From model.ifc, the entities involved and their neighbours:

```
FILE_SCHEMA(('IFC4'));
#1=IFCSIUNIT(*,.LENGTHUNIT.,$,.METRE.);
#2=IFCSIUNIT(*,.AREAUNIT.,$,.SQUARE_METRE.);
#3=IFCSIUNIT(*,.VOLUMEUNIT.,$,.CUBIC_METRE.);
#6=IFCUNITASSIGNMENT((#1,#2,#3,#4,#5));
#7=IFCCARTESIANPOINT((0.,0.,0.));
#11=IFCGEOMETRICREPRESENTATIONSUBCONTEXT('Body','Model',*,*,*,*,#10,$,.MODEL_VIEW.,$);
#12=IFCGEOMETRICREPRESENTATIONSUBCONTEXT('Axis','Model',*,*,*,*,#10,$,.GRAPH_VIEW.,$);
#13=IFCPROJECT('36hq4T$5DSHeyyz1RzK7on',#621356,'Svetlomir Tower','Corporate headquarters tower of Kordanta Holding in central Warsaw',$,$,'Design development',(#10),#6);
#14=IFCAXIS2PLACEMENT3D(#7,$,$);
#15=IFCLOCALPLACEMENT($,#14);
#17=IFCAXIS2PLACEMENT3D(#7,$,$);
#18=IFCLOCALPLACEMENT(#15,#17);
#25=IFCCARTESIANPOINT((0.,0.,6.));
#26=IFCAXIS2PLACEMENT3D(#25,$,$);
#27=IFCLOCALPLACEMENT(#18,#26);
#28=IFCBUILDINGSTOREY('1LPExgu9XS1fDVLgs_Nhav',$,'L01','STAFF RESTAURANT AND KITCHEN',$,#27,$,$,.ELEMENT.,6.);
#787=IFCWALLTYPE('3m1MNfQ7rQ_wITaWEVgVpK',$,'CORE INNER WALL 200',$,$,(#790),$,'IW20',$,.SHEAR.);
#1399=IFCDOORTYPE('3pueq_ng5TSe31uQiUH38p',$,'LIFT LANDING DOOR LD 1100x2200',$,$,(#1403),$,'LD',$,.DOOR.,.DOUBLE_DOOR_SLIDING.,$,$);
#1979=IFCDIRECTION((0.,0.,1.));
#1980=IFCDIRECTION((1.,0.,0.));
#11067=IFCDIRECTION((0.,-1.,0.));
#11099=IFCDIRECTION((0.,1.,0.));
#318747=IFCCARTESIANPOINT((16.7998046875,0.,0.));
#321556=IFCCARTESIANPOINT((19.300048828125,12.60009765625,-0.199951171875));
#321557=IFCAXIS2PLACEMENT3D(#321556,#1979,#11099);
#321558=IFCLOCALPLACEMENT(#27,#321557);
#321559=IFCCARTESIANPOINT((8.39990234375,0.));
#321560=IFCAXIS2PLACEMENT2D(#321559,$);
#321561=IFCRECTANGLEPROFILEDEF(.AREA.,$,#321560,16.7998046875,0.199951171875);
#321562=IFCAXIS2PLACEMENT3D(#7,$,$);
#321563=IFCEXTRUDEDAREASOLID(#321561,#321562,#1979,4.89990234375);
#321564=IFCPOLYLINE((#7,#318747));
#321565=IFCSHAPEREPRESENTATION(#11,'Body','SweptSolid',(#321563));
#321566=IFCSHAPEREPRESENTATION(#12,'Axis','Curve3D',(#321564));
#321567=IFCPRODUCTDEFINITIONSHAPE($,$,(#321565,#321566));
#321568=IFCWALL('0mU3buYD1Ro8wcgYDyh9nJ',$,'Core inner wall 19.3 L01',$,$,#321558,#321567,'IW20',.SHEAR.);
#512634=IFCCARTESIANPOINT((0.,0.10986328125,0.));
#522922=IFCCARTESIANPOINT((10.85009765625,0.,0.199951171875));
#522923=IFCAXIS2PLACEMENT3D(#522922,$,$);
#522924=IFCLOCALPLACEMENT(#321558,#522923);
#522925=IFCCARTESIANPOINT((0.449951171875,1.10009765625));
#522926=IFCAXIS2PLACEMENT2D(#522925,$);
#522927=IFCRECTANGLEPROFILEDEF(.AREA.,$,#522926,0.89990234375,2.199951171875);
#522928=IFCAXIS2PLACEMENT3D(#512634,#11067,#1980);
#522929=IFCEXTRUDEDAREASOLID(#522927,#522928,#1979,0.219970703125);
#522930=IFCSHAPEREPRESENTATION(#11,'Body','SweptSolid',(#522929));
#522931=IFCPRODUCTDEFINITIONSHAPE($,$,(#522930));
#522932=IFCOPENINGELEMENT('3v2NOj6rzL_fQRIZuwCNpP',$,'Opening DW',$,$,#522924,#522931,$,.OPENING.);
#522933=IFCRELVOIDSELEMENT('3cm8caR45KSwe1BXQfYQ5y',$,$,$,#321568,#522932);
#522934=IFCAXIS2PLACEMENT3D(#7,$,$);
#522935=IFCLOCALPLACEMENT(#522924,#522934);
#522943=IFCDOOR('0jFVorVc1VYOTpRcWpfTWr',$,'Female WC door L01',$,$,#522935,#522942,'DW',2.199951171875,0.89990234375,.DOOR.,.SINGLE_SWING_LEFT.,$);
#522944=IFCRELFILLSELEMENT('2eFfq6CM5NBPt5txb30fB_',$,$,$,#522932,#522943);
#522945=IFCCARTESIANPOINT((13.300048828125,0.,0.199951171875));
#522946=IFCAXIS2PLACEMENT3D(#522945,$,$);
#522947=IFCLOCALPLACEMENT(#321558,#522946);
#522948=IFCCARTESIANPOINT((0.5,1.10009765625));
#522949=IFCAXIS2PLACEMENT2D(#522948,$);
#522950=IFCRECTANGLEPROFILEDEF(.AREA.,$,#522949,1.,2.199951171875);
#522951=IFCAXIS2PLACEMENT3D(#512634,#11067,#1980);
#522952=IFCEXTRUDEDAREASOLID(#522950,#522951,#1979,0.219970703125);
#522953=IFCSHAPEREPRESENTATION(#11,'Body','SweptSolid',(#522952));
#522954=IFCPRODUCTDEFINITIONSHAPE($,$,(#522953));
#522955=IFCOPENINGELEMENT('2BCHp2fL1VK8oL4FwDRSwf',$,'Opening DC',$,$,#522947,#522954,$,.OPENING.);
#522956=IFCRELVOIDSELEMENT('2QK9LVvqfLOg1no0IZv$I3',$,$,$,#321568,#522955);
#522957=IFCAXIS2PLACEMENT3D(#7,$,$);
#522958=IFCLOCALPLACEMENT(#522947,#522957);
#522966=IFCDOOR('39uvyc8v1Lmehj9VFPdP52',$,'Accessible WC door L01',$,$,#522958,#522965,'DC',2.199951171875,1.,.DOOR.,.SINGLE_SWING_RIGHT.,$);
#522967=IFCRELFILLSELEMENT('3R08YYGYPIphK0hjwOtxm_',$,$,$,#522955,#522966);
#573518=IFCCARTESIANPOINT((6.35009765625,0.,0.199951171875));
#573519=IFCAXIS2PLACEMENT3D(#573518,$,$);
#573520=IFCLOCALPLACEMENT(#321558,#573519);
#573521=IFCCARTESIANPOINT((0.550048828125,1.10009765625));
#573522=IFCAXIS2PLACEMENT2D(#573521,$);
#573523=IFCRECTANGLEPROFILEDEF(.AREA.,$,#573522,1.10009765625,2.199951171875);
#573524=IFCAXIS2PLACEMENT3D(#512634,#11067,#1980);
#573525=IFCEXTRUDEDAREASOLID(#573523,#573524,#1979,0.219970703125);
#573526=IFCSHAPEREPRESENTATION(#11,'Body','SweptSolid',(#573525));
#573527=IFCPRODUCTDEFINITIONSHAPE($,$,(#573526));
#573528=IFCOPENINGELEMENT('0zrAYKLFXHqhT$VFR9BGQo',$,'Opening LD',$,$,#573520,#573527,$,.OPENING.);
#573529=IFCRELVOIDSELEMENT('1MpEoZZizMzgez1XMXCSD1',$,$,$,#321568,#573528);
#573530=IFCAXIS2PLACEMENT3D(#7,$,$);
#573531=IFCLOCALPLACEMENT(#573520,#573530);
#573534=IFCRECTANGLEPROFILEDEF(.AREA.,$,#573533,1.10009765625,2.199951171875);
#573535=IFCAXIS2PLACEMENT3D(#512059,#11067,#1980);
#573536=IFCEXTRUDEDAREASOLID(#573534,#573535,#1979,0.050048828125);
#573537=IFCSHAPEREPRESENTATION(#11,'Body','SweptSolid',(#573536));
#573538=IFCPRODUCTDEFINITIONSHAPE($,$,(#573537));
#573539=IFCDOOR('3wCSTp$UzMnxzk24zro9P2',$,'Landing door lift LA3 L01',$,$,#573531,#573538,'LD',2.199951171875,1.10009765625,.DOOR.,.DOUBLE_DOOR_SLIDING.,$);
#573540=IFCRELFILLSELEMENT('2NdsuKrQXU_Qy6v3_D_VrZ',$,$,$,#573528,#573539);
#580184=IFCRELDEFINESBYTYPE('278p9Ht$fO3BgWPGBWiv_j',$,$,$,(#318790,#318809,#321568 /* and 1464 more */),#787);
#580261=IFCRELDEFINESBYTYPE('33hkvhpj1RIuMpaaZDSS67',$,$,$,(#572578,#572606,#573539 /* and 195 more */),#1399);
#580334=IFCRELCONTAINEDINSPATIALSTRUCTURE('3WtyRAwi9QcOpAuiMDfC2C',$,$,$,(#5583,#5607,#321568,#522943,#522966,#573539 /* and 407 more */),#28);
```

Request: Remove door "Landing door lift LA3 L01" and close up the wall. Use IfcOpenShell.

```python
import ifcopenshell
import ifcopenshell.api.feature
import ifcopenshell.api.root
import ifcopenshell.geom
import ifcopenshell.util.shape

model = ifcopenshell.open("model.ifc")
settings = ifcopenshell.geom.settings()


def volume(element):
    """Net volume in cubic metres, openings subtracted."""
    shape = ifcopenshell.geom.create_shape(settings, element)
    return ifcopenshell.util.shape.get_volume(shape.geometry)


door = model.by_guid("3wCSTp$UzMnxzk24zro9P2")
opening = door.FillsVoids[0].RelatingOpeningElement
wall = opening.VoidsElements[0].RelatingBuildingElement
before = volume(wall)

ifcopenshell.api.root.remove_product(model, product=door)
ifcopenshell.api.feature.remove_feature(model, feature=opening)

after = volume(wall)

print(f"wall volume {before:.3f} -> {after:.3f} m3")

model.write("model_edited.ifc")
```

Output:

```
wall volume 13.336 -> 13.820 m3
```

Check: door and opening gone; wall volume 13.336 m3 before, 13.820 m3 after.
